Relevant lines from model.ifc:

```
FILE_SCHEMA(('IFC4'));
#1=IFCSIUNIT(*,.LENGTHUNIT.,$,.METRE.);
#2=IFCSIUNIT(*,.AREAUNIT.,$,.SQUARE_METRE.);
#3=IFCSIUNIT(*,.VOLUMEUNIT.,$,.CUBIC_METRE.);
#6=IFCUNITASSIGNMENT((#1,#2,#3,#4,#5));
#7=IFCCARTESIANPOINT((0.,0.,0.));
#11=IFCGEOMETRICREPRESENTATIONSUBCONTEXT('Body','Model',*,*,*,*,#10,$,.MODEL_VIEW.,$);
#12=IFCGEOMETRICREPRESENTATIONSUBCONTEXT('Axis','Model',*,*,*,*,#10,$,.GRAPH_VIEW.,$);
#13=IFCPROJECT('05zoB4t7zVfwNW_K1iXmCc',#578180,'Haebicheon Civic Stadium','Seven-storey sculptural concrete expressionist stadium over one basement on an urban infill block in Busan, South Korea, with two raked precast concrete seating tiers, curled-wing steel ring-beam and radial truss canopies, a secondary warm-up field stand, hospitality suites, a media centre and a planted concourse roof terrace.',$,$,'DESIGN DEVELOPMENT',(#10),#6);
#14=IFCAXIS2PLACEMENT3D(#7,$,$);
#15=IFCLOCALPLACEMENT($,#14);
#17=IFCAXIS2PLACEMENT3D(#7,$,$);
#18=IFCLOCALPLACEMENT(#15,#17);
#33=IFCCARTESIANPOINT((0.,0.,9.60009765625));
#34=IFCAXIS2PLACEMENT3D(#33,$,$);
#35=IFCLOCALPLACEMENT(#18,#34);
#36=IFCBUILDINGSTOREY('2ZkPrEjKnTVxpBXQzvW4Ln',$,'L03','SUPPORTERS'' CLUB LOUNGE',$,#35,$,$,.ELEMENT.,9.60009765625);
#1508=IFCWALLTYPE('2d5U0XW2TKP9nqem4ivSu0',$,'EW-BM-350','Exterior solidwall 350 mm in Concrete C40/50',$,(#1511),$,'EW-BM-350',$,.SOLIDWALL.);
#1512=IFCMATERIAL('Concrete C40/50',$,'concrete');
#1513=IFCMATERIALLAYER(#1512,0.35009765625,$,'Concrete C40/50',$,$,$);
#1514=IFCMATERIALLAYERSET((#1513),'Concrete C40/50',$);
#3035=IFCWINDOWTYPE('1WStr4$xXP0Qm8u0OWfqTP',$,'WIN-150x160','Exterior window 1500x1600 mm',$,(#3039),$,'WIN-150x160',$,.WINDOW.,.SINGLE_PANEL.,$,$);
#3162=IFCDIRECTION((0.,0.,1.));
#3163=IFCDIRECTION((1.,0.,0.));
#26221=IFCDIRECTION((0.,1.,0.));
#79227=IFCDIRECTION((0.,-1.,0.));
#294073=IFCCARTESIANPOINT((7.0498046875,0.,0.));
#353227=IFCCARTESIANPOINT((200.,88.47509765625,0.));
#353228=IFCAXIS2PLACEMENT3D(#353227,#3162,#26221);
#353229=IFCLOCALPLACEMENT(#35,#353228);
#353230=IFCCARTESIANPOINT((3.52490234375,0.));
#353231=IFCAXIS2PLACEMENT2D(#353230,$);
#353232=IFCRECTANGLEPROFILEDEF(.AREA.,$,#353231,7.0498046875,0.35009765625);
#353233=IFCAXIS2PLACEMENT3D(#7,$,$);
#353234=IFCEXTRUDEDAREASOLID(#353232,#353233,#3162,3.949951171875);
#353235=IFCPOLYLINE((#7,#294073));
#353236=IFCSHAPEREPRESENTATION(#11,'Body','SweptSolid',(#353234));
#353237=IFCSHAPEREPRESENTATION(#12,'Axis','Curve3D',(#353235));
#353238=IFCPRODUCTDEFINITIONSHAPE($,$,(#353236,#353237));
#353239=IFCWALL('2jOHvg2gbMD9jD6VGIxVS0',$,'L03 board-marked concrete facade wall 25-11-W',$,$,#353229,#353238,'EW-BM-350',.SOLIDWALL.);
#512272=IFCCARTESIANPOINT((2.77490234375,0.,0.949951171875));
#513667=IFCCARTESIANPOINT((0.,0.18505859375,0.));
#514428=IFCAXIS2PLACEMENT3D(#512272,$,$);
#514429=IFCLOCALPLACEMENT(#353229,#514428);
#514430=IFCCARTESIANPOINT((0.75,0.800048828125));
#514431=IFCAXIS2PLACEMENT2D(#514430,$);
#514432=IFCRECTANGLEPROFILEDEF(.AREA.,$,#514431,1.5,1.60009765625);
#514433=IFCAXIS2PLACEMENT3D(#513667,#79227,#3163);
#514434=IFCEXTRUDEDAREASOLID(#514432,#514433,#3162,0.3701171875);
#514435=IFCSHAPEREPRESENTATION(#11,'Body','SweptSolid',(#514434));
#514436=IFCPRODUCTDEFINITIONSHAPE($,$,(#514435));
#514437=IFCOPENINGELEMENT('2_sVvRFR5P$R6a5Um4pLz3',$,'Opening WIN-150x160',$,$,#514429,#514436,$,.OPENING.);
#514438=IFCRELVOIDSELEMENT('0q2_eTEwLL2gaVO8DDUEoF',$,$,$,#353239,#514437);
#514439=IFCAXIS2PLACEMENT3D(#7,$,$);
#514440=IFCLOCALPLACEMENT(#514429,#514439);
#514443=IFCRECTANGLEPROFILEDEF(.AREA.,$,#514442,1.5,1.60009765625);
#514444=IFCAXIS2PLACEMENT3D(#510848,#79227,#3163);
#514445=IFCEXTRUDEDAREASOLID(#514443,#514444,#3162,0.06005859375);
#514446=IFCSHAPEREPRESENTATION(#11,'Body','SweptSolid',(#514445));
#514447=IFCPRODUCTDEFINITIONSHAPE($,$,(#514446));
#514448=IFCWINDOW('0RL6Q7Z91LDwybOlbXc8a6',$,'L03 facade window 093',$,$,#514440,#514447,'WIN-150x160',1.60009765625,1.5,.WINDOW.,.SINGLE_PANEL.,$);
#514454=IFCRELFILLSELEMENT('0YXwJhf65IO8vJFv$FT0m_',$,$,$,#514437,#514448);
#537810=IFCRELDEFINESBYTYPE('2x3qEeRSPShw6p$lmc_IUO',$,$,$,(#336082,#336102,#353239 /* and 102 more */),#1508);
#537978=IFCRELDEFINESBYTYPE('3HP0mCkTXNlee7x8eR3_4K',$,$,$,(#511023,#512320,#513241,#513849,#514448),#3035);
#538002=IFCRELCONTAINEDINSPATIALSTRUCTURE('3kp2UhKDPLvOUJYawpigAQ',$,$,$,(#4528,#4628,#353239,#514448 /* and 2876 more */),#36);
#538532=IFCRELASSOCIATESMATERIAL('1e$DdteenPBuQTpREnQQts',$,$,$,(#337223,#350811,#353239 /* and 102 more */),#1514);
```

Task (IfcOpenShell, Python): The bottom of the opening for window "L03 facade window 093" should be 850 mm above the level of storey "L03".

```python
import numpy as np
import ifcopenshell
import ifcopenshell.api.geometry
import ifcopenshell.geom
import ifcopenshell.util.element
import ifcopenshell.util.placement
import ifcopenshell.util.shape
import ifcopenshell.util.unit

model = ifcopenshell.open("model.ifc")
unit_scale = ifcopenshell.util.unit.calculate_unit_scale(model)

window = model.by_guid("0RL6Q7Z91LDwybOlbXc8a6")
opening = window.FillsVoids[0].RelatingOpeningElement
storey = ifcopenshell.util.element.get_container(window, ifc_class="IfcBuildingStorey")
level = ifcopenshell.util.placement.get_local_placement(storey.ObjectPlacement)[2, 3]

# The opening's origin need not be at the sill, so measure its lowest point.
shape = ifcopenshell.geom.create_shape(ifcopenshell.geom.settings(), opening)
bottom = ifcopenshell.util.shape.get_shape_bottom_elevation(shape, shape.geometry) / unit_scale
dz = level + 0.85 / unit_scale - bottom

shift = np.array([0.0, 0.0, dz])
# The window is placed relative to its opening, so it follows when the opening moves.
matrix = ifcopenshell.util.placement.get_local_placement(opening.ObjectPlacement)
matrix[:3, 3] += shift
ifcopenshell.api.geometry.edit_object_placement(
    model, product=opening, matrix=matrix, is_si=False, should_transform_children=True
)

print(f"moved by {dz * unit_scale:+.3f} m")

model.write("model_v2.ifc")
```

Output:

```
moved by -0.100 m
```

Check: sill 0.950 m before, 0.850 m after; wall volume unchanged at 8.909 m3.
